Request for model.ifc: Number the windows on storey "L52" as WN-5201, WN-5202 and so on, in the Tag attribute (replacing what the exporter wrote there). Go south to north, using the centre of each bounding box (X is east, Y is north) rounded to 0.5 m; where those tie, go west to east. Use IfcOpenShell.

First a look at what the model holds.

```python
import ifcopenshell
import ifcopenshell.util.element
import ifcopenshell.util.placement

model = ifcopenshell.open("model.ifc")
print(model.schema)
storey = next(s for s in model.by_type("IfcBuildingStorey") if s.Name == "L52")
windows = [e for e in ifcopenshell.util.element.get_decomposition(storey) if e.is_a("IfcWindow")]
for e in sorted(windows, key=lambda e: e.id()):
    origin = ifcopenshell.util.placement.get_local_placement(e.ObjectPlacement)[:3, 3]
    print(e.id(), e.Tag, e.Name, origin.round(2) + 0.0, sep=" | ")
```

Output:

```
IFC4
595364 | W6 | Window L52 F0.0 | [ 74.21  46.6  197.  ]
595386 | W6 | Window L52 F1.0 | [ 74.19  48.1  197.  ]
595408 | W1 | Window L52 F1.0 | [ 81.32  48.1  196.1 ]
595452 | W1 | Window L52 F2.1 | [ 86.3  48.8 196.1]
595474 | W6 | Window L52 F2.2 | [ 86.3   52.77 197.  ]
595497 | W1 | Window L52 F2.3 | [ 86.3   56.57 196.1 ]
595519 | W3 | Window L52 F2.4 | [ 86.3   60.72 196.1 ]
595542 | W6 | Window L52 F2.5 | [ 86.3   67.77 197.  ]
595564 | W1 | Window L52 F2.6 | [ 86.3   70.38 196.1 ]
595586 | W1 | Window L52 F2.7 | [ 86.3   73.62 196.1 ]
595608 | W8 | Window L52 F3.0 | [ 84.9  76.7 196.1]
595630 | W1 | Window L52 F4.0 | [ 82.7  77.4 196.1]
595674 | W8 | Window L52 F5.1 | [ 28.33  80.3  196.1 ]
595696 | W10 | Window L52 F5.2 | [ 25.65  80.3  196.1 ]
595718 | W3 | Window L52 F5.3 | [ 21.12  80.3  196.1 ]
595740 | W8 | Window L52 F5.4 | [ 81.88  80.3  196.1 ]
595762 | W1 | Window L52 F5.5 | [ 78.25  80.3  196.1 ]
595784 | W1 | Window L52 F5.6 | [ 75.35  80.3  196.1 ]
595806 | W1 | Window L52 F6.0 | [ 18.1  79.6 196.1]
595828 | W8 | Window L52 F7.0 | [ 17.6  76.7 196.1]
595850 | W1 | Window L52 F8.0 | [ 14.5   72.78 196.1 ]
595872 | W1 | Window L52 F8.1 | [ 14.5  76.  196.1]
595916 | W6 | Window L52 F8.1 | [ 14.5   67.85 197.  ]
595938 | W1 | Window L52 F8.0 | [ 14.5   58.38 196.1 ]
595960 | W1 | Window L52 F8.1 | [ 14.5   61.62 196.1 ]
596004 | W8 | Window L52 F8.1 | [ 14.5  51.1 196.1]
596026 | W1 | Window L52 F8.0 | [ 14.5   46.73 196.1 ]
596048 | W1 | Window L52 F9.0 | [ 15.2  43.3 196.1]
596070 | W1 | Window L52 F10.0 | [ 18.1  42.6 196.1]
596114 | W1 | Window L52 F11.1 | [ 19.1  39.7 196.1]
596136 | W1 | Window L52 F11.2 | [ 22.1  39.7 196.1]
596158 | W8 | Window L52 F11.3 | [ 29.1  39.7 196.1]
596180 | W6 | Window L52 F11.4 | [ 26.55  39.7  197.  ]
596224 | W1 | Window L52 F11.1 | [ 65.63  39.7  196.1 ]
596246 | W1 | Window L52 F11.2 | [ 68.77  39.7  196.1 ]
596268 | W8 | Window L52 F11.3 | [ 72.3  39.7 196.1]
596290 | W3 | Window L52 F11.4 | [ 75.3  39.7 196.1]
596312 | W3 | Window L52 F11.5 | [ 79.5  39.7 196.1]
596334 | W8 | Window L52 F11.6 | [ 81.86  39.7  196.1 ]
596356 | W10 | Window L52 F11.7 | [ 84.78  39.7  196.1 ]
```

```python
import ifcopenshell
import ifcopenshell.geom
import ifcopenshell.util.element
import ifcopenshell.util.shape

model = ifcopenshell.open("model.ifc")
settings = ifcopenshell.geom.settings()
settings.set("use-world-coords", True)


def centre(element):
    shape = ifcopenshell.geom.create_shape(settings, element)
    return ifcopenshell.util.shape.get_bbox_centroid(shape.geometry)


storey = next(s for s in model.by_type("IfcBuildingStorey") if s.Name == "L52")
windows = [e for e in ifcopenshell.util.element.get_decomposition(storey) if e.is_a("IfcWindow")]

# Insertion points can sit at a corner or the storey origin, so sort by the geometry (in metres).
centres = {e: centre(e) for e in windows}
windows.sort(key=lambda e: (round(centres[e][1] / 0.5), centres[e][0]))

for i, e in enumerate(windows, start=1):
    number = f"WN-52{i:02d}"
    e.Tag = number
    print(e.id(), number)

model.write("model_v2.ifc")
```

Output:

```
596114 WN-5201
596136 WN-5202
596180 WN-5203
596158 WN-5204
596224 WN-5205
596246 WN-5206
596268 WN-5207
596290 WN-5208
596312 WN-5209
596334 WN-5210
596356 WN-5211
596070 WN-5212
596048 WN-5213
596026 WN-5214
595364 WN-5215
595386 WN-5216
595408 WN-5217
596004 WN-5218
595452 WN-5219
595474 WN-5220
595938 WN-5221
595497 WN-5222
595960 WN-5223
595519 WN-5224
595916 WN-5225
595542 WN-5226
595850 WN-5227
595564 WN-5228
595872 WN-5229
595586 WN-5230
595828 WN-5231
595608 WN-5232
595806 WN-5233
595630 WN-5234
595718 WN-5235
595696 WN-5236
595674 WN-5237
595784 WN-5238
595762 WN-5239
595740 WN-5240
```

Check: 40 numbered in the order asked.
